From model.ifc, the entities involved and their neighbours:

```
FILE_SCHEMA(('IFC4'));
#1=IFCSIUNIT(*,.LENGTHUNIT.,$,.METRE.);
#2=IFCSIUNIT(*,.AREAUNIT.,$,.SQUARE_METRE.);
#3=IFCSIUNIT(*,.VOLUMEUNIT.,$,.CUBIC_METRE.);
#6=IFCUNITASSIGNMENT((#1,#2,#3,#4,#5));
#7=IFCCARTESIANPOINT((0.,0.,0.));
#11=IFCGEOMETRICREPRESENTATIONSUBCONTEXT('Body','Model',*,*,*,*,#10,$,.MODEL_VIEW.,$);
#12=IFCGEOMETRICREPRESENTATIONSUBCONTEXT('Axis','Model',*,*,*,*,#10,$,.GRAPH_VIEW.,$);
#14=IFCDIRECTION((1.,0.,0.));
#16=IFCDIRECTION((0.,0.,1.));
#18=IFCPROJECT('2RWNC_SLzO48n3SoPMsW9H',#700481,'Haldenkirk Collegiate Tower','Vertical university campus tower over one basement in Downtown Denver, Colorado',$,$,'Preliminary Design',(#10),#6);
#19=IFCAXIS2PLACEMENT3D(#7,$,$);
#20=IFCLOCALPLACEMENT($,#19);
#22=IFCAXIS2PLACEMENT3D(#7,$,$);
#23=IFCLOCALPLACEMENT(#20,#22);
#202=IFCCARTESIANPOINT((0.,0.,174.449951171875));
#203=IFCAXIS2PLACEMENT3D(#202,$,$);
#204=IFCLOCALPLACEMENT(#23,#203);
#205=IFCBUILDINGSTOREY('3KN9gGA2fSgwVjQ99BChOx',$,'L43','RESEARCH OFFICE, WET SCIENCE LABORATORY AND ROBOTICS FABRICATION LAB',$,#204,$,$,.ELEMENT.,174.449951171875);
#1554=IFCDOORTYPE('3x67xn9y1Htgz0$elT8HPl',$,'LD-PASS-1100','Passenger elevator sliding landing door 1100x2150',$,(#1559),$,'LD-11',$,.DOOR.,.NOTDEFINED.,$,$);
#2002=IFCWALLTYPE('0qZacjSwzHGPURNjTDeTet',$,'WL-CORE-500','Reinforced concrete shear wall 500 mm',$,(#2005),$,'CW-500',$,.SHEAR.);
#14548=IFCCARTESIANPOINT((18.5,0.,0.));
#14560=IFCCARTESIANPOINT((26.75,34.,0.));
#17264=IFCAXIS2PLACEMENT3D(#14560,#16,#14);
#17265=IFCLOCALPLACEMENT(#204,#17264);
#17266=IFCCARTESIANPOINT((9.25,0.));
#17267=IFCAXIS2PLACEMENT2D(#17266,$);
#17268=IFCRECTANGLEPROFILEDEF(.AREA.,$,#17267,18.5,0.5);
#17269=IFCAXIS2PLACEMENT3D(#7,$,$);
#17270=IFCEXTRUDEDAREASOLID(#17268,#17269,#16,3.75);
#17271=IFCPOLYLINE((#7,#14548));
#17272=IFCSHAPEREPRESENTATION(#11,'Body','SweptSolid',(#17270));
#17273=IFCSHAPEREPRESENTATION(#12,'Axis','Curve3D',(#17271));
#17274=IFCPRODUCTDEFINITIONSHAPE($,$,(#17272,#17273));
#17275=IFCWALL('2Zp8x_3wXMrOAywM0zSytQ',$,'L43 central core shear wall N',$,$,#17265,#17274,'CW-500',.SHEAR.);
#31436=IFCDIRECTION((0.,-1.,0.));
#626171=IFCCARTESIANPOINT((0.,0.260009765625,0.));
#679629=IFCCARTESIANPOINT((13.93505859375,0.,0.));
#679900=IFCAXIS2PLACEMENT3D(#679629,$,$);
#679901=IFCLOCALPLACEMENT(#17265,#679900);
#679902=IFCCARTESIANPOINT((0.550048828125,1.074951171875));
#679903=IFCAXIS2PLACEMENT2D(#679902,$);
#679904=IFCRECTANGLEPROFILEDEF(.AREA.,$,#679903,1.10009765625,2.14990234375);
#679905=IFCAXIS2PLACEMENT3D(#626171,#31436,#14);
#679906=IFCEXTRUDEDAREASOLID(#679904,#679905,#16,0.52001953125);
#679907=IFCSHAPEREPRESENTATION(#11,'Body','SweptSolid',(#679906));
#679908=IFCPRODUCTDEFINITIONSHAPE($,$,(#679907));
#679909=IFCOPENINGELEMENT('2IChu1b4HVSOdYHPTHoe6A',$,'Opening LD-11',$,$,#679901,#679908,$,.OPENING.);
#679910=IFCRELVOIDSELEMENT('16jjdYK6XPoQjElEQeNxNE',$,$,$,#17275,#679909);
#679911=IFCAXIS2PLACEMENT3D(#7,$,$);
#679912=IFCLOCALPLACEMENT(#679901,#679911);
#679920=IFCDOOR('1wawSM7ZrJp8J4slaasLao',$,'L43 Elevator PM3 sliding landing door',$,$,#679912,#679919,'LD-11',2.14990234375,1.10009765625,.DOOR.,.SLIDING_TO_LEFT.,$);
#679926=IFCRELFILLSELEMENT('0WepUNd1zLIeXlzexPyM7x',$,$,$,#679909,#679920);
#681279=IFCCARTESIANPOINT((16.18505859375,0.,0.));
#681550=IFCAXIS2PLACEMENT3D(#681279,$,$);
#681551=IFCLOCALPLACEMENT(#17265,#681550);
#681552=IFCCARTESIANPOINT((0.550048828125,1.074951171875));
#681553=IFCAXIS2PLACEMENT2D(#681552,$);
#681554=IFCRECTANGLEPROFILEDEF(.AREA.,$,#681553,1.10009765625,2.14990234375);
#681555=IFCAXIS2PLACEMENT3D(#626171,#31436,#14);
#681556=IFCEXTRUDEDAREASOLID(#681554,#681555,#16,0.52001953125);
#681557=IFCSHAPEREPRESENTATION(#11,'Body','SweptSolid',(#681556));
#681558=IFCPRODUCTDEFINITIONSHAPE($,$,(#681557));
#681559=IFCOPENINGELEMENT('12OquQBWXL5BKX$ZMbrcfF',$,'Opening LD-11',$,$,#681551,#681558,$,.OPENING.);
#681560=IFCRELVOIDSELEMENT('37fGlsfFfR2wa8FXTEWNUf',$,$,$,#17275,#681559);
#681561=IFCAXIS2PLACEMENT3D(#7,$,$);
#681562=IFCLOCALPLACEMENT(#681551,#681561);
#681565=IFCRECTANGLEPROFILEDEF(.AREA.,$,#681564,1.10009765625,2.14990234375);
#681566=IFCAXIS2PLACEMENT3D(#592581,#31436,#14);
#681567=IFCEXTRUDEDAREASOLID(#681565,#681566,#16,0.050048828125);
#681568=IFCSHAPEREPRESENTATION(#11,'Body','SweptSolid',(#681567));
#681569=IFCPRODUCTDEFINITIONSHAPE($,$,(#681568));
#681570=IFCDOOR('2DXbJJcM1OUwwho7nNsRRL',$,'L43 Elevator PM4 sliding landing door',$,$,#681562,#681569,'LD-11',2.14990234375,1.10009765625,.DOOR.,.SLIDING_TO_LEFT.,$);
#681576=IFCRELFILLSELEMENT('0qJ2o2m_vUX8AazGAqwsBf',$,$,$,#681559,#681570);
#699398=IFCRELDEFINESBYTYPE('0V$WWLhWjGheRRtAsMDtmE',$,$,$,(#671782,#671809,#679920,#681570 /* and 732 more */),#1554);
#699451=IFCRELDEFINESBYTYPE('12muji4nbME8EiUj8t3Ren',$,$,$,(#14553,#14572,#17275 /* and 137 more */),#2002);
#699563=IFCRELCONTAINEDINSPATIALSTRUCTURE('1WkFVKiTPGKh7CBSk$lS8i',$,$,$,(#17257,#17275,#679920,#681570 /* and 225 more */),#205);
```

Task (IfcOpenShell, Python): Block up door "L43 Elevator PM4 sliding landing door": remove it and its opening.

```python
import ifcopenshell
import ifcopenshell.api.feature
import ifcopenshell.api.root
import ifcopenshell.geom
import ifcopenshell.util.shape

model = ifcopenshell.open("model.ifc")
settings = ifcopenshell.geom.settings()


def volume(element):
    """Net volume in cubic metres, openings subtracted."""
    shape = ifcopenshell.geom.create_shape(settings, element)
    return ifcopenshell.util.shape.get_volume(shape.geometry)


door = model.by_guid("2DXbJJcM1OUwwho7nNsRRL")
opening = door.FillsVoids[0].RelatingOpeningElement
wall = opening.VoidsElements[0].RelatingBuildingElement
before = volume(wall)

ifcopenshell.api.root.remove_product(model, product=door)
ifcopenshell.api.feature.remove_feature(model, feature=opening)

after = volume(wall)

print(f"wall volume {before:.3f} -> {after:.3f} m3")

model.write("model_rev.ifc")
```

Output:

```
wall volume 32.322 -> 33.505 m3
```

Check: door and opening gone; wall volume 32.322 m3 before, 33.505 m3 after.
